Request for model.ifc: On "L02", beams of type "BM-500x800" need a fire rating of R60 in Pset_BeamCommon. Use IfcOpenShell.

First a look at what the model holds.

```python
import ifcopenshell
import ifcopenshell.util.element

model = ifcopenshell.open("model.ifc")
print(model.schema)
storey = next(s for s in model.by_type("IfcBuildingStorey") if s.Name == "L02")
beams = [e for e in ifcopenshell.util.element.get_decomposition(storey) if e.is_a("IfcBeam")]
seen = {}
for e in beams:
    element_type = ifcopenshell.util.element.get_type(e)
    key = (element_type.Name if element_type != e and element_type else None, ifcopenshell.util.element.get_pset(e, "Pset_BeamCommon", "FireRating"))
    seen[key] = seen.get(key, 0) + 1
for (name, value), count in sorted(seen.items(), key=str):
    print(count, "x", name, "|", value)
```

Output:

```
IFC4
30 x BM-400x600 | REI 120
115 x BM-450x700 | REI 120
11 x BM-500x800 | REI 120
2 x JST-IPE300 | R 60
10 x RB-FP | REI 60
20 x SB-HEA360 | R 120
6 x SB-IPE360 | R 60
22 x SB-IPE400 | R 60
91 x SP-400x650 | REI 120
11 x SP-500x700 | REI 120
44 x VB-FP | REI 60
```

```python
import ifcopenshell
import ifcopenshell.api.pset
import ifcopenshell.util.element

model = ifcopenshell.open("model.ifc")

storey = next(s for s in model.by_type("IfcBuildingStorey") if s.Name == "L02")
beams = [e for e in ifcopenshell.util.element.get_decomposition(storey) if e.is_a("IfcBeam")]

count = 0
for e in beams:
    element_type = ifcopenshell.util.element.get_type(e)
    if element_type in (None, e) or element_type.Name != "BM-500x800":
        continue
    # add_pset returns the element's existing set when there is one.
    pset = ifcopenshell.api.pset.add_pset(model, product=e, name="Pset_BeamCommon")
    ifcopenshell.api.pset.edit_pset(model, pset=pset, properties={"FireRating": "R60"})
    count += 1

print(count, "beams updated")

model.write("model_rev.ifc")
```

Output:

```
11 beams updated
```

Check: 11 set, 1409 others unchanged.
